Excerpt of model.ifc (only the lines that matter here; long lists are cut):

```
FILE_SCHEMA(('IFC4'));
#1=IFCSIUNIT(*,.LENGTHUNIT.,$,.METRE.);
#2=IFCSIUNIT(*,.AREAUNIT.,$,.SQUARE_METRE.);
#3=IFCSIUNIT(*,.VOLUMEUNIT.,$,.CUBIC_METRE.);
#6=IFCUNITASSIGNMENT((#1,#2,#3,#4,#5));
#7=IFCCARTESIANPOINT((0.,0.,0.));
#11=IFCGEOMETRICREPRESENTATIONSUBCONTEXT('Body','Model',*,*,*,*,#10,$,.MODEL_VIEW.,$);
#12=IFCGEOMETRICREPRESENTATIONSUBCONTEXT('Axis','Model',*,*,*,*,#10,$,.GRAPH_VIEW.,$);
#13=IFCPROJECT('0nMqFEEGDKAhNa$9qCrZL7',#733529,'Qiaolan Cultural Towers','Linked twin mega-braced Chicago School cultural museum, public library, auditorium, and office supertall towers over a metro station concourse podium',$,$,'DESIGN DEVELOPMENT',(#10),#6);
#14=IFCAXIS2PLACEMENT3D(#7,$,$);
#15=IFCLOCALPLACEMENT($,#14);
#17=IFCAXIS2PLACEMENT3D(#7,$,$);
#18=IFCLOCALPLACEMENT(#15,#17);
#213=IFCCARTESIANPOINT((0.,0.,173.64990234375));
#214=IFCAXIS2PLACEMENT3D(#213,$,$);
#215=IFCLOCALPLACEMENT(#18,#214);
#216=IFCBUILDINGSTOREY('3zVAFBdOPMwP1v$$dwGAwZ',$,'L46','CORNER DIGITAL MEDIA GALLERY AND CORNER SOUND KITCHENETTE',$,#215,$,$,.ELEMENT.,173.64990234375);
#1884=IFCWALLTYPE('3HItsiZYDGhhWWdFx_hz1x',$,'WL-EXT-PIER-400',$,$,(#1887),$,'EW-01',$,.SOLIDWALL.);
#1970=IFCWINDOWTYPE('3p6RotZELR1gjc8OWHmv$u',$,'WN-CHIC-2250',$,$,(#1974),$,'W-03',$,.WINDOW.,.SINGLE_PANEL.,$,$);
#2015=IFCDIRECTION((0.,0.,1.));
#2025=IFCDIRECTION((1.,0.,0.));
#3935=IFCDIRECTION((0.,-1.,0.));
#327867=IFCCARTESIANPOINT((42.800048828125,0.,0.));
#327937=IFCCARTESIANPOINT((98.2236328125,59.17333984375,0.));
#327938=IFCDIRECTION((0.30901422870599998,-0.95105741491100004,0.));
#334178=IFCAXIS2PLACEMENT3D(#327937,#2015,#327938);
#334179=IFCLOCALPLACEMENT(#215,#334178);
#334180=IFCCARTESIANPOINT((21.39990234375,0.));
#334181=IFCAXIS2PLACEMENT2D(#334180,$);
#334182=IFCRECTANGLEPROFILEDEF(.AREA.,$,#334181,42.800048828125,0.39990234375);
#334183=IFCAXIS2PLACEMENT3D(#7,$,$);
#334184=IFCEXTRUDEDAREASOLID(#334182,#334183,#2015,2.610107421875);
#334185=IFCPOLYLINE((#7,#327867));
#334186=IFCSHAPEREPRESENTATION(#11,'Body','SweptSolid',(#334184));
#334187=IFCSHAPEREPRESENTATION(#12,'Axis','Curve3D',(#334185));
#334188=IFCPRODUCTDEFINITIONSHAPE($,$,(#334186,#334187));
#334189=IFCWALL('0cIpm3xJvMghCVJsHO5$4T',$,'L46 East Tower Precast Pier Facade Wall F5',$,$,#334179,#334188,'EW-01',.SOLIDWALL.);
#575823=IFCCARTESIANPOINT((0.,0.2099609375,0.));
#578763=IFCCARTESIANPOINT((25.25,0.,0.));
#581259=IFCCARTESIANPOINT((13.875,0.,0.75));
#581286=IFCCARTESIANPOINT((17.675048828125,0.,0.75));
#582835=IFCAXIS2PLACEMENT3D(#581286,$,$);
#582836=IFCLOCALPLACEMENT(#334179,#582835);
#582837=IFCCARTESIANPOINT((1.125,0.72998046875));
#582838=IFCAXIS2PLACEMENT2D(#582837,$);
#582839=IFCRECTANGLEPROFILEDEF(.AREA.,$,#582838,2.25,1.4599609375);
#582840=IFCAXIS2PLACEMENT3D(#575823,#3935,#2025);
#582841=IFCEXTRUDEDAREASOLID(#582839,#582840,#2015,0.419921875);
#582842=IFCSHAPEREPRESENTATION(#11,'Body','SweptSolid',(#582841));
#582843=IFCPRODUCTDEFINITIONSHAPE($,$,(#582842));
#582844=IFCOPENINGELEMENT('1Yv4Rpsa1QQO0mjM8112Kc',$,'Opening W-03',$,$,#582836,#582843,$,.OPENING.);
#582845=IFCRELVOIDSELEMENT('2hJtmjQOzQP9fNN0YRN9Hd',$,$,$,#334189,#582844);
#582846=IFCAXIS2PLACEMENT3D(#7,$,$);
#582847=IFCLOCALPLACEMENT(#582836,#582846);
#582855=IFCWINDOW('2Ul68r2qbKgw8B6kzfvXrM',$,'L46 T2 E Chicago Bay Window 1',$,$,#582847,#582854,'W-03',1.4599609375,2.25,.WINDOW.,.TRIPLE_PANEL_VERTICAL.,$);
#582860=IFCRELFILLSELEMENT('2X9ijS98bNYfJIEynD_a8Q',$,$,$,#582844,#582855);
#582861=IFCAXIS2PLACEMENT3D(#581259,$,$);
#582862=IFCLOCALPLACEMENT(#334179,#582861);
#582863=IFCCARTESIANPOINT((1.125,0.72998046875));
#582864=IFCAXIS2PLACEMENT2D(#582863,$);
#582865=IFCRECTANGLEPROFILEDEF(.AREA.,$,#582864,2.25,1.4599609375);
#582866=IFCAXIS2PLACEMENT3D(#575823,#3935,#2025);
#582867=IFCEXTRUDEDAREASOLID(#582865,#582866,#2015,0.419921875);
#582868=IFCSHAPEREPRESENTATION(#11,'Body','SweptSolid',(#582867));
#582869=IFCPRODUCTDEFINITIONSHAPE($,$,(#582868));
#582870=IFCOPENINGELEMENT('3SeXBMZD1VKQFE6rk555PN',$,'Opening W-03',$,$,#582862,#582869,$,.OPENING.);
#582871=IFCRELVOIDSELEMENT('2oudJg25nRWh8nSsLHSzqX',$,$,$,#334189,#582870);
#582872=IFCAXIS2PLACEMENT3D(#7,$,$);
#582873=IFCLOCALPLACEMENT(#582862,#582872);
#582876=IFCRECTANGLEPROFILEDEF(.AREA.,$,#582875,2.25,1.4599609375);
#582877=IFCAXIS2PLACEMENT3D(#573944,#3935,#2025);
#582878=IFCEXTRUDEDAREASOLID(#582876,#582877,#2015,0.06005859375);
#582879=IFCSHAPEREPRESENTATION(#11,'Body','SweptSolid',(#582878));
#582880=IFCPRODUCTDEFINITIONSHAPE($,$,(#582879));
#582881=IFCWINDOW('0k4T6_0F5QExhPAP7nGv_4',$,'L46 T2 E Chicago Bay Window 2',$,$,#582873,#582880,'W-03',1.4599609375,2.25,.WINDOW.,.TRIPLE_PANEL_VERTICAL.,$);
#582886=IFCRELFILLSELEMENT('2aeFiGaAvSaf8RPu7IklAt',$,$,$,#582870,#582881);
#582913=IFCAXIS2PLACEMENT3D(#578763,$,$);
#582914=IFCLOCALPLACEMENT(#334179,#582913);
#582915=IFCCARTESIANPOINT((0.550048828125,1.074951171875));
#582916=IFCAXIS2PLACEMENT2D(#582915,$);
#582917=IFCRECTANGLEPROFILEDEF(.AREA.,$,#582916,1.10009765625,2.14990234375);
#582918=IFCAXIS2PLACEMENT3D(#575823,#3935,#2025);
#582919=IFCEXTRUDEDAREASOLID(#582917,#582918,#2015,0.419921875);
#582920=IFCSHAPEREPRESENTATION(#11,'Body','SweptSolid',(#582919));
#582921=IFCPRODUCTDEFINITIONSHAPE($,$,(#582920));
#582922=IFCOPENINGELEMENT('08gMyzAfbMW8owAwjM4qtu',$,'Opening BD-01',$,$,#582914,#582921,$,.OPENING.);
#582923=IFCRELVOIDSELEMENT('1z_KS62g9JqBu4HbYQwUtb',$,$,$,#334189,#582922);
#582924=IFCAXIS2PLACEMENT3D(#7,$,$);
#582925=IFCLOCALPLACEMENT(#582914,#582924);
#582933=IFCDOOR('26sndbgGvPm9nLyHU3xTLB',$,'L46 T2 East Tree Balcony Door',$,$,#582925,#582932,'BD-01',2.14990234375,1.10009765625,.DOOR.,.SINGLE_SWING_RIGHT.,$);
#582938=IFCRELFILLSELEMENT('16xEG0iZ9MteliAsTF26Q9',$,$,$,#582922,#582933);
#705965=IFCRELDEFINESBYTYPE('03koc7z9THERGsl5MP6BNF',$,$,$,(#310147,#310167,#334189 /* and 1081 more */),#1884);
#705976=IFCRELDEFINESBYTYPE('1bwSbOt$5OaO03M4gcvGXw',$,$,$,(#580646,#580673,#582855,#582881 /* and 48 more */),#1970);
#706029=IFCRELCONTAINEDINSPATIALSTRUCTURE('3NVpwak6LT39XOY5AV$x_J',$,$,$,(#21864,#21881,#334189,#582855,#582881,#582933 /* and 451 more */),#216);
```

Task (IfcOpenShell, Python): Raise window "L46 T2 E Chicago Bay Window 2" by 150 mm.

```python
import numpy as np
import ifcopenshell
import ifcopenshell.api.geometry
import ifcopenshell.util.placement
import ifcopenshell.util.unit

model = ifcopenshell.open("model.ifc")
unit_scale = ifcopenshell.util.unit.calculate_unit_scale(model)

window = model.by_id(582881)
opening = window.FillsVoids[0].RelatingOpeningElement
dz = 0.15

shift = np.array([0.0, 0.0, dz])
# The window is placed relative to its opening, so it follows when the opening moves.
matrix = ifcopenshell.util.placement.get_local_placement(opening.ObjectPlacement)
matrix[:3, 3] += shift
ifcopenshell.api.geometry.edit_object_placement(
    model, product=opening, matrix=matrix, is_si=False, should_transform_children=True
)

print(f"moved by {dz * unit_scale:+.3f} m")

model.write("model_v2.ifc")
```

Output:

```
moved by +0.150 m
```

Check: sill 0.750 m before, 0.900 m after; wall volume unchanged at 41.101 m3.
